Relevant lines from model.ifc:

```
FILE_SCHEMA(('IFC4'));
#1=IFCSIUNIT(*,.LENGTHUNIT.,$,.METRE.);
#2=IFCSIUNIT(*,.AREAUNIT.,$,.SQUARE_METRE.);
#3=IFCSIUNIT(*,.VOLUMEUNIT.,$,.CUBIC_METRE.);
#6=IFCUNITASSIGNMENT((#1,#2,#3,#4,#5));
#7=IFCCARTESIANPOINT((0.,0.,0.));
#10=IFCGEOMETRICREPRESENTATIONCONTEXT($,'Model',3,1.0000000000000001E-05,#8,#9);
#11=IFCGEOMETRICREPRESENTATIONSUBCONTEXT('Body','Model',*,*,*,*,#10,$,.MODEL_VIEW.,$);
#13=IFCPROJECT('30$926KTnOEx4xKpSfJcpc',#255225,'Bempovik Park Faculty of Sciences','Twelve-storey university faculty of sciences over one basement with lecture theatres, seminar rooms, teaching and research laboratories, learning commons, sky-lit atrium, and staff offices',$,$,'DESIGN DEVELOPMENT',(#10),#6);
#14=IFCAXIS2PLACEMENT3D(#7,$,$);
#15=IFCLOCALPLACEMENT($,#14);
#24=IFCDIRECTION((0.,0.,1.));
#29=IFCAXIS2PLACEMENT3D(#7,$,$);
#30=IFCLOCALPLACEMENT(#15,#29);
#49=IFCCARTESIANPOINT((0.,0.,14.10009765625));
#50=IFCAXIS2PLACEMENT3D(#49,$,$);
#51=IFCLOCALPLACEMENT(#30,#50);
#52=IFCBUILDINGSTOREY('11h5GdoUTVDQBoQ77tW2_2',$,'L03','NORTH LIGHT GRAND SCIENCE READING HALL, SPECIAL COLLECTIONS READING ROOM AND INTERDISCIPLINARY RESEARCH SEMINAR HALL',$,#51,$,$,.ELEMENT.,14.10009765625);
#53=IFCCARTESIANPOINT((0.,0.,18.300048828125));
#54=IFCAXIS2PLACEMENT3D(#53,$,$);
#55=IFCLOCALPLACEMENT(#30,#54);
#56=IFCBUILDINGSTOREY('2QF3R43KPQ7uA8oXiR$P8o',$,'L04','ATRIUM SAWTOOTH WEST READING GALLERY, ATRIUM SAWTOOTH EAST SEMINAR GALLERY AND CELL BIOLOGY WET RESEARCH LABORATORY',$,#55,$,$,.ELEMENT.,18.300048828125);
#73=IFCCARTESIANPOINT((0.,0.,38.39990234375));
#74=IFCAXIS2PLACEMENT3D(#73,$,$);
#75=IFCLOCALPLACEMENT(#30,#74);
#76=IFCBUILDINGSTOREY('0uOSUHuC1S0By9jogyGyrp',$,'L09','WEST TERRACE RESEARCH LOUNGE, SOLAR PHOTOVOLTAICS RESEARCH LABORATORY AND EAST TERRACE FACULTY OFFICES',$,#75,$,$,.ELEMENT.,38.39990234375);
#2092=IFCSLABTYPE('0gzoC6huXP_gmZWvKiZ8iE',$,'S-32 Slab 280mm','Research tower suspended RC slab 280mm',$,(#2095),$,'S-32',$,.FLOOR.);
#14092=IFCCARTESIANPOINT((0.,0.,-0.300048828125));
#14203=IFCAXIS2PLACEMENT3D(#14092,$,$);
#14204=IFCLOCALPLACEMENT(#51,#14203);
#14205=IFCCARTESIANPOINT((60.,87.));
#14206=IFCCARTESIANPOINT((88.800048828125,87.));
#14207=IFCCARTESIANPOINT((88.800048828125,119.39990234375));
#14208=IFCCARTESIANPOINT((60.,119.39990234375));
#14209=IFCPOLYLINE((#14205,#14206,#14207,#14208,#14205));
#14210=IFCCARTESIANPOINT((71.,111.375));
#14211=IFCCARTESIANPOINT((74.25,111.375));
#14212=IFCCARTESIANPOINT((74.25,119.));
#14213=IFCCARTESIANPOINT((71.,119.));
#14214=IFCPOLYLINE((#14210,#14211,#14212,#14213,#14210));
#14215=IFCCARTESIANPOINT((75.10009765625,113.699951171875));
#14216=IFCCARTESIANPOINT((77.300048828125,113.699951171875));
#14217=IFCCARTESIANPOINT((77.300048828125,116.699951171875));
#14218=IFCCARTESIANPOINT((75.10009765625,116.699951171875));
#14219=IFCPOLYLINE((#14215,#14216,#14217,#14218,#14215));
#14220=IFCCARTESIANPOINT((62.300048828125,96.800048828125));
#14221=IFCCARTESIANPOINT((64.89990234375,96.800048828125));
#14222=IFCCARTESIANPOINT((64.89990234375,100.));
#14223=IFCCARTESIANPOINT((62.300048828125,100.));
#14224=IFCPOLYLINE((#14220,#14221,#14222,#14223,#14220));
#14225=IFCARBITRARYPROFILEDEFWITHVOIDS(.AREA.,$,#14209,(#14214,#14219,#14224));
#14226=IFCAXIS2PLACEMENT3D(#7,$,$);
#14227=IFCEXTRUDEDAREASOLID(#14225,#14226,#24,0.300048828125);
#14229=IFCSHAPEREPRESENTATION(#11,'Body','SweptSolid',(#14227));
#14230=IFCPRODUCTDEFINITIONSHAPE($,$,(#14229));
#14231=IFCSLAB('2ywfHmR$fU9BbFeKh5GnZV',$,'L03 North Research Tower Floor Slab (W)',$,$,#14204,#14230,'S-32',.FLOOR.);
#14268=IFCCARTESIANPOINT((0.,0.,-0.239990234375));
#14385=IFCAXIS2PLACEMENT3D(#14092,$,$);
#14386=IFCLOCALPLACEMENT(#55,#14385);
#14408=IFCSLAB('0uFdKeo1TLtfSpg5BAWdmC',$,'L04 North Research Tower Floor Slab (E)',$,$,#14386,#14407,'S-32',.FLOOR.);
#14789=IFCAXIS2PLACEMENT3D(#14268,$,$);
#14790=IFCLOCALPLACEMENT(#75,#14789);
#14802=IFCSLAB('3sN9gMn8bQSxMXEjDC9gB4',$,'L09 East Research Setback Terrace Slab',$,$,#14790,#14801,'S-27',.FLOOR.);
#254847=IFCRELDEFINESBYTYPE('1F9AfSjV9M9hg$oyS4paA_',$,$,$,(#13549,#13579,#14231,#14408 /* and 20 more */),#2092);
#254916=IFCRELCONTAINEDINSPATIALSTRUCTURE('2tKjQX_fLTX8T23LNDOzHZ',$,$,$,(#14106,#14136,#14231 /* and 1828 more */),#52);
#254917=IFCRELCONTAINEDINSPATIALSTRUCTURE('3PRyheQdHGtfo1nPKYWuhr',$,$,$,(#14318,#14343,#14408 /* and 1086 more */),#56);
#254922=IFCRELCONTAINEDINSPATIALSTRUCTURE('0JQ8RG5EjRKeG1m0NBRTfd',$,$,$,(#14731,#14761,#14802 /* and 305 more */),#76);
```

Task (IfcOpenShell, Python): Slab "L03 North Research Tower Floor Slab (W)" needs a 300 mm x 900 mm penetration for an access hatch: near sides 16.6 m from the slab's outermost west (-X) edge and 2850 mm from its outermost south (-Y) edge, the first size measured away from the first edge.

```python
import numpy as np
import ifcopenshell
import ifcopenshell.api.feature
import ifcopenshell.api.geometry
import ifcopenshell.api.root
import ifcopenshell.geom
import ifcopenshell.util.placement
import ifcopenshell.util.representation
import ifcopenshell.util.shape
import ifcopenshell.util.unit

model = ifcopenshell.open("model.ifc")
unit_scale = ifcopenshell.util.unit.calculate_unit_scale(model)
settings = ifcopenshell.geom.settings()


def volume(element):
    """Net volume in cubic metres, openings subtracted."""
    shape = ifcopenshell.geom.create_shape(settings, element)
    return ifcopenshell.util.shape.get_volume(shape.geometry)


slab = model.by_id(14231)
before = volume(slab)

# Extent in the slab's own axes, in metres. The edges named are its -X and -Y sides.
slab_shape = ifcopenshell.geom.create_shape(settings, slab)
vertices = ifcopenshell.util.shape.get_vertices(slab_shape.geometry)
x_min, y_min, bottom = vertices.min(axis=0)
top = vertices[:, 2].max()

opening = ifcopenshell.api.root.create_entity(model, ifc_class="IfcOpeningElement", name="Access hatch opening", predefined_type="OPENING")
context = ifcopenshell.util.representation.get_context(model, "Model", "Body", "MODEL_VIEW")
width, depth = 0.3, 0.9
outline = [(0.0, 0.0), (width, 0.0), (width, depth), (0.0, depth), (0.0, 0.0)]
# Overshoot both faces by 50 mm so the cut is clean.
shape = ifcopenshell.api.geometry.add_slab_representation(
    model, context=context, depth=top - bottom + 0.1, polyline=outline
)
ifcopenshell.api.geometry.assign_representation(model, product=opening, representation=shape)

matrix = ifcopenshell.util.placement.get_local_placement(slab.ObjectPlacement)
matrix[:, 3] = matrix @ np.append(np.array([x_min + 16.6, y_min + 2.85, bottom - 0.05]) / unit_scale, 1.0)
ifcopenshell.api.geometry.edit_object_placement(model, product=opening, matrix=matrix, is_si=False)
ifcopenshell.api.feature.add_feature(model, feature=opening, element=slab)

after = volume(slab)

print(f"slab volume {before:.3f} -> {after:.3f} m3")

model.write("model_updated.ifc")
```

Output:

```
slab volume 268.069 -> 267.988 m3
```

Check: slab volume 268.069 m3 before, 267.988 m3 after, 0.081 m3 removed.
